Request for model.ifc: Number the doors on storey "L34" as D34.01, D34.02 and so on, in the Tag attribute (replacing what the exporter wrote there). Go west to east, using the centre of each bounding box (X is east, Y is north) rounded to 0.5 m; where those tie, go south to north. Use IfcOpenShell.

First a look at what the model holds.

```python
import ifcopenshell
import ifcopenshell.util.element
import ifcopenshell.util.placement

model = ifcopenshell.open("model.ifc")
print(model.schema)
storey = next(s for s in model.by_type("IfcBuildingStorey") if s.Name == "L34")
doors = [e for e in ifcopenshell.util.element.get_decomposition(storey) if e.is_a("IfcDoor")]
for e in sorted(doors, key=lambda e: e.id()):
    origin = ifcopenshell.util.placement.get_local_placement(e.ObjectPlacement)[:3, 3]
    print(e.id(), e.Tag, e.Name, origin.round(2) + 0.0, sep=" | ")
```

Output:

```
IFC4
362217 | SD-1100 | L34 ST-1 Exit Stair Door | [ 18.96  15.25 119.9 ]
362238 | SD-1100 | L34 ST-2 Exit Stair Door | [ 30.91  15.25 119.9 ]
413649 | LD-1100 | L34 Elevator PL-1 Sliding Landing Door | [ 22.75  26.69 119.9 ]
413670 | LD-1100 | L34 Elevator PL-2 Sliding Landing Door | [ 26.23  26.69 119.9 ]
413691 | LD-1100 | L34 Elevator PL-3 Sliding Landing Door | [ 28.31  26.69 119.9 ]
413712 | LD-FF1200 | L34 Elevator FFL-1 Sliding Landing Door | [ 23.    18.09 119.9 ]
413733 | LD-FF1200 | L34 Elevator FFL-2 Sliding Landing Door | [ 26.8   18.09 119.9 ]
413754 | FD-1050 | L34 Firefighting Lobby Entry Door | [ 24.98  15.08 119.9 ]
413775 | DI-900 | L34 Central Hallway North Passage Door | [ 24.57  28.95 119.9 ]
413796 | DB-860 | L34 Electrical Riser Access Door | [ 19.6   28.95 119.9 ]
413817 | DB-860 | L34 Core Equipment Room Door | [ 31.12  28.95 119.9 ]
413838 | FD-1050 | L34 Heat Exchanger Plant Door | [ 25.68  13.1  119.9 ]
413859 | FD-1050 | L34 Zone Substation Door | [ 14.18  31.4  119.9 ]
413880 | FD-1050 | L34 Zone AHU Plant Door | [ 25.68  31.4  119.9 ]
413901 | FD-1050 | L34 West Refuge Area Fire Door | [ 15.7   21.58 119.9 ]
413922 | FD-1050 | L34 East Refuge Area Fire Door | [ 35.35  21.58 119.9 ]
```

```python
import ifcopenshell
import ifcopenshell.geom
import ifcopenshell.util.element
import ifcopenshell.util.shape

model = ifcopenshell.open("model.ifc")
settings = ifcopenshell.geom.settings()
settings.set("use-world-coords", True)


def centre(element):
    shape = ifcopenshell.geom.create_shape(settings, element)
    return ifcopenshell.util.shape.get_bbox_centroid(shape.geometry)


storey = next(s for s in model.by_type("IfcBuildingStorey") if s.Name == "L34")
doors = [e for e in ifcopenshell.util.element.get_decomposition(storey) if e.is_a("IfcDoor")]

# Insertion points can sit at a corner or the storey origin, so sort by the geometry (in metres).
centres = {e: centre(e) for e in doors}
doors.sort(key=lambda e: (round(centres[e][0] / 0.5), centres[e][1]))

for i, e in enumerate(doors, start=1):
    number = f"D34.{i:02d}"
    e.Tag = number
    print(e.id(), number)

model.write("model_rev.ifc")
```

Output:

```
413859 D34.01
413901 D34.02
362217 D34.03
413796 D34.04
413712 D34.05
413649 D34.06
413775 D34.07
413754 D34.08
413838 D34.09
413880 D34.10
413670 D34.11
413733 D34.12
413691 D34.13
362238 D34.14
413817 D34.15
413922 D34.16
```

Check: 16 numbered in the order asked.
